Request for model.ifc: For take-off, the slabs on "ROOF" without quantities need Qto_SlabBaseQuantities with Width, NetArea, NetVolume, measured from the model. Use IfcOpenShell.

First a look at what the model holds.

```python
import ifcopenshell
import ifcopenshell.util.element
import ifcopenshell.util.unit

model = ifcopenshell.open("model.ifc")
print(model.schema)
for unit_type in ("LENGTHUNIT", "AREAUNIT", "VOLUMEUNIT"):
    print(unit_type, ifcopenshell.util.unit.calculate_unit_scale(model, unit_type))
storey = next(s for s in model.by_type("IfcBuildingStorey") if s.Name == "ROOF")
slabs = [e for e in ifcopenshell.util.element.get_decomposition(storey) if e.is_a("IfcSlab")]
for e in sorted(slabs, key=lambda e: e.id()):
    print(e.id(), e.is_a(), e.Name, list(ifcopenshell.util.element.get_psets(e, qtos_only=True)), sep=" | ")
```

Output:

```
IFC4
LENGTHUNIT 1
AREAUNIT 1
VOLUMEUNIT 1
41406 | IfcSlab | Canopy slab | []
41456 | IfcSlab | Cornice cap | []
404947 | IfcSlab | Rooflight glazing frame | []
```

```python
import ifcopenshell
import ifcopenshell.api.pset
import ifcopenshell.geom
import ifcopenshell.util.element
import ifcopenshell.util.shape
import ifcopenshell.util.unit

model = ifcopenshell.open("model.ifc")
unit_scale = ifcopenshell.util.unit.calculate_unit_scale(model)
area_scale = ifcopenshell.util.unit.calculate_unit_scale(model, "AREAUNIT")
volume_scale = ifcopenshell.util.unit.calculate_unit_scale(model, "VOLUMEUNIT")
settings = ifcopenshell.geom.settings()

storey = next(s for s in model.by_type("IfcBuildingStorey") if s.Name == "ROOF")
slabs = [e for e in ifcopenshell.util.element.get_decomposition(storey) if e.is_a("IfcSlab")]

for e in sorted(slabs, key=lambda e: e.id()):
    if ifcopenshell.util.element.get_psets(e, qtos_only=True, should_inherit=False):
        continue
    # Geometry comes back in metres, in the element's own axes.
    shape = ifcopenshell.geom.create_shape(settings, e)
    values = {
        "Width": ifcopenshell.util.shape.get_z(shape.geometry) / unit_scale,
        "NetArea": ifcopenshell.util.shape.get_footprint_area(shape.geometry) / area_scale,
        "NetVolume": ifcopenshell.util.shape.get_volume(shape.geometry) / volume_scale,
    }
    qto = ifcopenshell.api.pset.add_qto(model, product=e, name="Qto_SlabBaseQuantities")
    ifcopenshell.api.pset.edit_qto(model, qto=qto, properties=values)
    print(e.id(), {k: round(v, 3) for k, v in values.items()})

model.write("model_rev.ifc")
```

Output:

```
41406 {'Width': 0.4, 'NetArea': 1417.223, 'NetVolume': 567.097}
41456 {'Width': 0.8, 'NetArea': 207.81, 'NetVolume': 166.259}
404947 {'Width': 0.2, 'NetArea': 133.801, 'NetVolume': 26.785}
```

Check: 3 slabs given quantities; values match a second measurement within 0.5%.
